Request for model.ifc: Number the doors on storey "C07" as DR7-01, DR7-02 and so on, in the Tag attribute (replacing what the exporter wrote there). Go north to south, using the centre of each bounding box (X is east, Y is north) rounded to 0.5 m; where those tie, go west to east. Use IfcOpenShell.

First a look at what the model holds.

```python
import ifcopenshell
import ifcopenshell.util.element
import ifcopenshell.util.placement

model = ifcopenshell.open("model.ifc")
print(model.schema)
storey = next(s for s in model.by_type("IfcBuildingStorey") if s.Name == "C07")
doors = [e for e in ifcopenshell.util.element.get_decomposition(storey) if e.is_a("IfcDoor")]
for e in sorted(doors, key=lambda e: e.id()):
    origin = ifcopenshell.util.placement.get_local_placement(e.ObjectPlacement)[:3, 3]
    print(e.id(), e.Tag, e.Name, origin.round(2) + 0.0, sep=" | ")
```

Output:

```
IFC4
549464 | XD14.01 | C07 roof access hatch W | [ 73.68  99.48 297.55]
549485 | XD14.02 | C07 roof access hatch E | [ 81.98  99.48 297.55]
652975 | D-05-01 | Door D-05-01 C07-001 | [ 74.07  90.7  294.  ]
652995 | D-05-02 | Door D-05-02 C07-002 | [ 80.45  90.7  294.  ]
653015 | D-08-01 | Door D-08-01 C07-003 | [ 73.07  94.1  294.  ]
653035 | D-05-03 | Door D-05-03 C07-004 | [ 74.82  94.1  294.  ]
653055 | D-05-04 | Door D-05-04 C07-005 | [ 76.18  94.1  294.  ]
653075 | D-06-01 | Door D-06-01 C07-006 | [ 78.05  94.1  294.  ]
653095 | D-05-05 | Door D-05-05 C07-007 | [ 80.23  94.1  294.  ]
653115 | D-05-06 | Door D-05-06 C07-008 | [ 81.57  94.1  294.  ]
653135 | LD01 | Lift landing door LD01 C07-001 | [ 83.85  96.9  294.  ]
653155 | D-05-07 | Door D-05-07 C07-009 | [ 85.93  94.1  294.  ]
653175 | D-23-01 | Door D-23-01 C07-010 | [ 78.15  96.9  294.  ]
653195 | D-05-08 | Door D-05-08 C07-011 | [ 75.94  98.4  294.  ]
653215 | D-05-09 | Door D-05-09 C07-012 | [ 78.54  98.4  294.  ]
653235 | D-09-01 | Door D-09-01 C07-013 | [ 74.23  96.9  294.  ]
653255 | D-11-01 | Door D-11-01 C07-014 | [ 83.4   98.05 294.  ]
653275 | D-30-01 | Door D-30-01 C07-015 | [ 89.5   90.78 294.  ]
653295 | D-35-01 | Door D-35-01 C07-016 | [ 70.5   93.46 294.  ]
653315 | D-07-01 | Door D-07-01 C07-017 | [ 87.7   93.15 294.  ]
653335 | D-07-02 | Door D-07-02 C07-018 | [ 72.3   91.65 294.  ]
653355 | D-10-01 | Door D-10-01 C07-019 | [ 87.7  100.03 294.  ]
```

```python
import ifcopenshell
import ifcopenshell.geom
import ifcopenshell.util.element
import ifcopenshell.util.shape

model = ifcopenshell.open("model.ifc")
settings = ifcopenshell.geom.settings()
settings.set("use-world-coords", True)


def centre(element):
    shape = ifcopenshell.geom.create_shape(settings, element)
    return ifcopenshell.util.shape.get_bbox_centroid(shape.geometry)


storey = next(s for s in model.by_type("IfcBuildingStorey") if s.Name == "C07")
doors = [e for e in ifcopenshell.util.element.get_decomposition(storey) if e.is_a("IfcDoor")]

# Insertion points can sit at a corner or the storey origin, so sort by the geometry (in metres).
centres = {e: centre(e) for e in doors}
doors.sort(key=lambda e: (-round(centres[e][1] / 0.5), centres[e][0]))

for i, e in enumerate(doors, start=1):
    number = f"DR7-{i:02d}"
    e.Tag = number
    print(e.id(), number)

model.write("model_v2.ifc")
```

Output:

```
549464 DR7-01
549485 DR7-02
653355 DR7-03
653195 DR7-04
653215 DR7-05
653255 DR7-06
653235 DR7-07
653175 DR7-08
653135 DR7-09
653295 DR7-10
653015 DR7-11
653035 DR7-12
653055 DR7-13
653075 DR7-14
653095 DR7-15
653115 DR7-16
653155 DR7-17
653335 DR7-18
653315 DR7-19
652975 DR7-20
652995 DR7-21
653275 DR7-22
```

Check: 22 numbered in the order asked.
